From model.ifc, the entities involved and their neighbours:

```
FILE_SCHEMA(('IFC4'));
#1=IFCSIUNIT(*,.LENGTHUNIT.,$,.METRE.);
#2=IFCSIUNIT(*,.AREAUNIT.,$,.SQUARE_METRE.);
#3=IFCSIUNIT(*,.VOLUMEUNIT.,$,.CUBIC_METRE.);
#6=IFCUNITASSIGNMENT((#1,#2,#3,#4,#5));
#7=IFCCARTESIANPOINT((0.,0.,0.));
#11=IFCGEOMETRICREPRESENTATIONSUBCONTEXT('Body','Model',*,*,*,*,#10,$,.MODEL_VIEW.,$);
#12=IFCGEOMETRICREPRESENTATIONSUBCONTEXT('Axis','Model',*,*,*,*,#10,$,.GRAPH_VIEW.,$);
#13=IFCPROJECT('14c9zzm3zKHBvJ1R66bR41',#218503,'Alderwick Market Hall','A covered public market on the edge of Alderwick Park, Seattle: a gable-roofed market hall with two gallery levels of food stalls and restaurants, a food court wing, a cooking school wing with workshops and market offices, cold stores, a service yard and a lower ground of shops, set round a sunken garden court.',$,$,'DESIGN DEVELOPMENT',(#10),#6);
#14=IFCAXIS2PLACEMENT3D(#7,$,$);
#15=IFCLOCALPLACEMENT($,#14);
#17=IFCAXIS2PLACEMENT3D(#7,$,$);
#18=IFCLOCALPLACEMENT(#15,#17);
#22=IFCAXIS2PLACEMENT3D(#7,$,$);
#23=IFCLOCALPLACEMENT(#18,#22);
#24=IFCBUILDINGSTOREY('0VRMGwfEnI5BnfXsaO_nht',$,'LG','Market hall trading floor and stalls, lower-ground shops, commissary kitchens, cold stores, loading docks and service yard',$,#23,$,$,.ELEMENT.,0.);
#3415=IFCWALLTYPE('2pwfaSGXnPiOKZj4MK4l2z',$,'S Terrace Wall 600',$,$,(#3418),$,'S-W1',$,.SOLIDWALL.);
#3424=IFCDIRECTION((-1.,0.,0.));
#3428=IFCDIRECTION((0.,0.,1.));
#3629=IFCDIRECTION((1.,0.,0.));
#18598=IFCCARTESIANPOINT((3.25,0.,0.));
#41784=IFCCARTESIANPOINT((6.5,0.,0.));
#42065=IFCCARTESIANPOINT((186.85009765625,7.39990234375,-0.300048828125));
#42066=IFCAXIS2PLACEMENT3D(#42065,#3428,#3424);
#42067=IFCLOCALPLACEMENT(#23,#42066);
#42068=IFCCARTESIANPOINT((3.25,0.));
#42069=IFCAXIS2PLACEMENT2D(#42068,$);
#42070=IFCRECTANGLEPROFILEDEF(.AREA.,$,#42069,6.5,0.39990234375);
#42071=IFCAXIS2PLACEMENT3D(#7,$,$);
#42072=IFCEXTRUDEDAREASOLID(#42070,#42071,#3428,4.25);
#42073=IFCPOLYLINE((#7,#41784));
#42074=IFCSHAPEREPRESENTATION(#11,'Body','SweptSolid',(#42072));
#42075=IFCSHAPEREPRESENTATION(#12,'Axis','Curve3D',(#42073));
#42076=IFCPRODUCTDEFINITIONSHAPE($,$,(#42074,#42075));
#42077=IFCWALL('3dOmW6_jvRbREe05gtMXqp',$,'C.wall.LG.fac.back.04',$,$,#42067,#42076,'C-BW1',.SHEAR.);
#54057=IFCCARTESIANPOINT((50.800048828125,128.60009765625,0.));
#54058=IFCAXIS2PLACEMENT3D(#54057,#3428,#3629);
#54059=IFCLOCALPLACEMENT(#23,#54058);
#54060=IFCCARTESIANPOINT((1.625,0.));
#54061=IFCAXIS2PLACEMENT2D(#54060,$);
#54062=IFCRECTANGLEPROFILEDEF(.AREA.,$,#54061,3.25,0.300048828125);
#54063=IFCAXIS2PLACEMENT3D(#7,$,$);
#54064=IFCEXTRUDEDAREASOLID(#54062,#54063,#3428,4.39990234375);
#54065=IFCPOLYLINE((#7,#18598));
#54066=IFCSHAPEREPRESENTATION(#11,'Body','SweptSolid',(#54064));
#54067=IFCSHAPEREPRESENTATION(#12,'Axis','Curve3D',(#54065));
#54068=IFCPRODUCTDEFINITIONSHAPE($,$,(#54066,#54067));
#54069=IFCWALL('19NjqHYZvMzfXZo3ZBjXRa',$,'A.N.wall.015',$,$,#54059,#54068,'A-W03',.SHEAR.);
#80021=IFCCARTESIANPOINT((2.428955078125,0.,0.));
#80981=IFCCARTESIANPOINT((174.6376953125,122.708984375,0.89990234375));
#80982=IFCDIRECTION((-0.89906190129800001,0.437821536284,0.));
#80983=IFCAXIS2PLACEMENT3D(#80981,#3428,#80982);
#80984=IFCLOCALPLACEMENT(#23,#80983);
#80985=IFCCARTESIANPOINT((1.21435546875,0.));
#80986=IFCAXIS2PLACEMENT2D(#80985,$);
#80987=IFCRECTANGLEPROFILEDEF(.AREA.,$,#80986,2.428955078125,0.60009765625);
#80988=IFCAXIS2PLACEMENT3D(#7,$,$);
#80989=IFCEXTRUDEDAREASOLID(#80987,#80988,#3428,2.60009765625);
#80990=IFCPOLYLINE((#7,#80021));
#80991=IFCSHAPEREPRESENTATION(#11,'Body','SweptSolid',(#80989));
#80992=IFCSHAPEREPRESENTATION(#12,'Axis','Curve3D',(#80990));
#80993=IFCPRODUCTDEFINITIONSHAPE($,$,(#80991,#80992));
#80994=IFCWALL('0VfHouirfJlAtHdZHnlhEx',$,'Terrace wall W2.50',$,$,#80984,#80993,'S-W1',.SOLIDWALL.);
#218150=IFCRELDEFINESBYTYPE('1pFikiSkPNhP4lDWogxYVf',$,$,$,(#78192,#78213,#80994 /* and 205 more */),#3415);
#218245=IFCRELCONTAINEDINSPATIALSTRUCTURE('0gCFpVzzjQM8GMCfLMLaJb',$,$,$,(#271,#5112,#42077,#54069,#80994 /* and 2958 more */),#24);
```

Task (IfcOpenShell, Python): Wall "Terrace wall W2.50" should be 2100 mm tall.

```python
import ifcopenshell
import ifcopenshell.geom
import ifcopenshell.util.representation
import ifcopenshell.util.shape
import ifcopenshell.util.unit

model = ifcopenshell.open("model.ifc")
unit_scale = ifcopenshell.util.unit.calculate_unit_scale(model)
settings = ifcopenshell.geom.settings()


def volume(element):
    """Net volume in cubic metres, openings subtracted."""
    shape = ifcopenshell.geom.create_shape(settings, element)
    return ifcopenshell.util.shape.get_volume(shape.geometry)


wall = model.by_guid("0VfHouirfJlAtHdZHnlhEx")
before = volume(wall)

body = ifcopenshell.util.representation.get_representation(wall, "Model", "Body")
solid = body.Items[0]
old_height = solid.Depth
solid.Depth = 2.1 / unit_scale
after = volume(wall)

print(f"height {old_height:g} -> {solid.Depth:g}, volume {before:.3f} -> {after:.3f} m3")

model.write("model-out.ifc")
```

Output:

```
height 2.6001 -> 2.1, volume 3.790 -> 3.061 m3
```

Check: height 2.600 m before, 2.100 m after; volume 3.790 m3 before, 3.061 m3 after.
